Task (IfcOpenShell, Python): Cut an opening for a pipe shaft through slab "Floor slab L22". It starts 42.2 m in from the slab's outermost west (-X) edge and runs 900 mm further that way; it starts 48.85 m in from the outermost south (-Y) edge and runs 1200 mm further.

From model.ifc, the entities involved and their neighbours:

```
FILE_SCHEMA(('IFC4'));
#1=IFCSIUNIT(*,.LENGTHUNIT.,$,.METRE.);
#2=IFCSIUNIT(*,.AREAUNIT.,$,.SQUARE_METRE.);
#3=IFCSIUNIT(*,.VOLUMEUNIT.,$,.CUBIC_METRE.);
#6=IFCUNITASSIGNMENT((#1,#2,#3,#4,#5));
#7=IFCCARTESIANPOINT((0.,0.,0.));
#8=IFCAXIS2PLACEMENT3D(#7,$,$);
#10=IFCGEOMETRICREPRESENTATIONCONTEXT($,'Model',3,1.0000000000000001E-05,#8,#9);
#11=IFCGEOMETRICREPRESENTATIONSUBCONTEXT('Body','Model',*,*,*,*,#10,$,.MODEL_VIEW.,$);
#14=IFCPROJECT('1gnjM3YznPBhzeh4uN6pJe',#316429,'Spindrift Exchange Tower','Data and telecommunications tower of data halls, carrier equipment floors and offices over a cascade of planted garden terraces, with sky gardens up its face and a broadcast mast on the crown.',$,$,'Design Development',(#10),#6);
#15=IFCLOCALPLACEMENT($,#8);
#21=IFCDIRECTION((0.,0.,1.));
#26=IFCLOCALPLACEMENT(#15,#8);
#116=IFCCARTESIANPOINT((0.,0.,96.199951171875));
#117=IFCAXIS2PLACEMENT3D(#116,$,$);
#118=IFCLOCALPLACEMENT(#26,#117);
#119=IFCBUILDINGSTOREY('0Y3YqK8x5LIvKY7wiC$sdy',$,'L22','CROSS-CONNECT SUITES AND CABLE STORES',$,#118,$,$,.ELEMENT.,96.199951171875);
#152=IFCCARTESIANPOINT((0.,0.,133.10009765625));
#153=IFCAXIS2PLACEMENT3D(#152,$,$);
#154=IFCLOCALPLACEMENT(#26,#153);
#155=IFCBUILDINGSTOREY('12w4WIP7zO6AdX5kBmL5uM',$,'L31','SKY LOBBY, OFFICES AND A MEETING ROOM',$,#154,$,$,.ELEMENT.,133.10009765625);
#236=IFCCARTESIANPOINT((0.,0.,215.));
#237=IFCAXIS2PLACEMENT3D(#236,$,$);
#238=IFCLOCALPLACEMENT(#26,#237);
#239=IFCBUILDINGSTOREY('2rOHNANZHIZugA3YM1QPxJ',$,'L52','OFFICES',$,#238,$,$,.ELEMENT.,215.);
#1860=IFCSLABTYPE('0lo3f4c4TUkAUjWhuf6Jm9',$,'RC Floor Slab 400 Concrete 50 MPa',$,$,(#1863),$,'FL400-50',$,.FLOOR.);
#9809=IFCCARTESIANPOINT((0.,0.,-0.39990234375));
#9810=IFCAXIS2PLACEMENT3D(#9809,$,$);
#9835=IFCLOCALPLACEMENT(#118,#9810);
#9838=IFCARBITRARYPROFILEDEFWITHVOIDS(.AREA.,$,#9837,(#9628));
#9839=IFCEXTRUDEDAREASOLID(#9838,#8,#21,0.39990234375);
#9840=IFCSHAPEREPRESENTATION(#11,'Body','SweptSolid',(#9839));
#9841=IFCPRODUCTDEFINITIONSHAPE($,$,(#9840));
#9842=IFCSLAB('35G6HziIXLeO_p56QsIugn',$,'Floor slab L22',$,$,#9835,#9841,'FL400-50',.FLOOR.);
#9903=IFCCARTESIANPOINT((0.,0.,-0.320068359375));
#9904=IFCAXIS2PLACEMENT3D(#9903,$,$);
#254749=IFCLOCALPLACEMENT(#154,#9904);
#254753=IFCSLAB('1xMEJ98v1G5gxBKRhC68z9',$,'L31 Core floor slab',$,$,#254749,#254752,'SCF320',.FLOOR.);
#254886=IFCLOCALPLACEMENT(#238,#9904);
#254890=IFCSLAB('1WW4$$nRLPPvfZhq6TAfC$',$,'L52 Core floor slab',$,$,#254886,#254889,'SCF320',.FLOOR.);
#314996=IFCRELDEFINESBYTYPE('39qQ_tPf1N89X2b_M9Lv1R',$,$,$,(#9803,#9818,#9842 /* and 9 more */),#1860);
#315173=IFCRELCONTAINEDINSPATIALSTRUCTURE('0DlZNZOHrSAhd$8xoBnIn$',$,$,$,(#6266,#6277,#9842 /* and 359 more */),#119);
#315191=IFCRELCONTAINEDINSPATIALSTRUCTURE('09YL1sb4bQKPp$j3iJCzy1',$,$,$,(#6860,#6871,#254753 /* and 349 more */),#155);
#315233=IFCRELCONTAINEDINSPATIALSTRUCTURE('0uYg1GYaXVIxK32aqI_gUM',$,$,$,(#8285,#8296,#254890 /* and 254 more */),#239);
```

```python
import numpy as np
import ifcopenshell
import ifcopenshell.api.feature
import ifcopenshell.api.geometry
import ifcopenshell.api.root
import ifcopenshell.geom
import ifcopenshell.util.placement
import ifcopenshell.util.representation
import ifcopenshell.util.shape
import ifcopenshell.util.unit

model = ifcopenshell.open("model.ifc")
unit_scale = ifcopenshell.util.unit.calculate_unit_scale(model)
settings = ifcopenshell.geom.settings()


def volume(element):
    """Net volume in cubic metres, openings subtracted."""
    shape = ifcopenshell.geom.create_shape(settings, element)
    return ifcopenshell.util.shape.get_volume(shape.geometry)


slab = model.by_guid("35G6HziIXLeO_p56QsIugn")
before = volume(slab)

# Extent in the slab's own axes, in metres. The edges named are its -X and -Y sides.
slab_shape = ifcopenshell.geom.create_shape(settings, slab)
vertices = ifcopenshell.util.shape.get_vertices(slab_shape.geometry)
x_min, y_min, bottom = vertices.min(axis=0)
top = vertices[:, 2].max()

opening = ifcopenshell.api.root.create_entity(model, ifc_class="IfcOpeningElement", name="Pipe shaft opening", predefined_type="OPENING")
context = ifcopenshell.util.representation.get_context(model, "Model", "Body", "MODEL_VIEW")
width, depth = 0.9, 1.2
outline = [(0.0, 0.0), (width, 0.0), (width, depth), (0.0, depth), (0.0, 0.0)]
# Overshoot both faces by 50 mm so the cut is clean.
shape = ifcopenshell.api.geometry.add_slab_representation(
    model, context=context, depth=top - bottom + 0.1, polyline=outline
)
ifcopenshell.api.geometry.assign_representation(model, product=opening, representation=shape)

matrix = ifcopenshell.util.placement.get_local_placement(slab.ObjectPlacement)
matrix[:, 3] = matrix @ np.append(np.array([x_min + 42.2, y_min + 48.85, bottom - 0.05]) / unit_scale, 1.0)
ifcopenshell.api.geometry.edit_object_placement(model, product=opening, matrix=matrix, is_si=False)
ifcopenshell.api.feature.add_feature(model, feature=opening, element=slab)

after = volume(slab)

print(f"slab volume {before:.3f} -> {after:.3f} m3")

model.write("model_v2.ifc")
```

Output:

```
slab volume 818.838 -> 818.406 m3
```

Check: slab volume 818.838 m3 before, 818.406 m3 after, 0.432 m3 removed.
